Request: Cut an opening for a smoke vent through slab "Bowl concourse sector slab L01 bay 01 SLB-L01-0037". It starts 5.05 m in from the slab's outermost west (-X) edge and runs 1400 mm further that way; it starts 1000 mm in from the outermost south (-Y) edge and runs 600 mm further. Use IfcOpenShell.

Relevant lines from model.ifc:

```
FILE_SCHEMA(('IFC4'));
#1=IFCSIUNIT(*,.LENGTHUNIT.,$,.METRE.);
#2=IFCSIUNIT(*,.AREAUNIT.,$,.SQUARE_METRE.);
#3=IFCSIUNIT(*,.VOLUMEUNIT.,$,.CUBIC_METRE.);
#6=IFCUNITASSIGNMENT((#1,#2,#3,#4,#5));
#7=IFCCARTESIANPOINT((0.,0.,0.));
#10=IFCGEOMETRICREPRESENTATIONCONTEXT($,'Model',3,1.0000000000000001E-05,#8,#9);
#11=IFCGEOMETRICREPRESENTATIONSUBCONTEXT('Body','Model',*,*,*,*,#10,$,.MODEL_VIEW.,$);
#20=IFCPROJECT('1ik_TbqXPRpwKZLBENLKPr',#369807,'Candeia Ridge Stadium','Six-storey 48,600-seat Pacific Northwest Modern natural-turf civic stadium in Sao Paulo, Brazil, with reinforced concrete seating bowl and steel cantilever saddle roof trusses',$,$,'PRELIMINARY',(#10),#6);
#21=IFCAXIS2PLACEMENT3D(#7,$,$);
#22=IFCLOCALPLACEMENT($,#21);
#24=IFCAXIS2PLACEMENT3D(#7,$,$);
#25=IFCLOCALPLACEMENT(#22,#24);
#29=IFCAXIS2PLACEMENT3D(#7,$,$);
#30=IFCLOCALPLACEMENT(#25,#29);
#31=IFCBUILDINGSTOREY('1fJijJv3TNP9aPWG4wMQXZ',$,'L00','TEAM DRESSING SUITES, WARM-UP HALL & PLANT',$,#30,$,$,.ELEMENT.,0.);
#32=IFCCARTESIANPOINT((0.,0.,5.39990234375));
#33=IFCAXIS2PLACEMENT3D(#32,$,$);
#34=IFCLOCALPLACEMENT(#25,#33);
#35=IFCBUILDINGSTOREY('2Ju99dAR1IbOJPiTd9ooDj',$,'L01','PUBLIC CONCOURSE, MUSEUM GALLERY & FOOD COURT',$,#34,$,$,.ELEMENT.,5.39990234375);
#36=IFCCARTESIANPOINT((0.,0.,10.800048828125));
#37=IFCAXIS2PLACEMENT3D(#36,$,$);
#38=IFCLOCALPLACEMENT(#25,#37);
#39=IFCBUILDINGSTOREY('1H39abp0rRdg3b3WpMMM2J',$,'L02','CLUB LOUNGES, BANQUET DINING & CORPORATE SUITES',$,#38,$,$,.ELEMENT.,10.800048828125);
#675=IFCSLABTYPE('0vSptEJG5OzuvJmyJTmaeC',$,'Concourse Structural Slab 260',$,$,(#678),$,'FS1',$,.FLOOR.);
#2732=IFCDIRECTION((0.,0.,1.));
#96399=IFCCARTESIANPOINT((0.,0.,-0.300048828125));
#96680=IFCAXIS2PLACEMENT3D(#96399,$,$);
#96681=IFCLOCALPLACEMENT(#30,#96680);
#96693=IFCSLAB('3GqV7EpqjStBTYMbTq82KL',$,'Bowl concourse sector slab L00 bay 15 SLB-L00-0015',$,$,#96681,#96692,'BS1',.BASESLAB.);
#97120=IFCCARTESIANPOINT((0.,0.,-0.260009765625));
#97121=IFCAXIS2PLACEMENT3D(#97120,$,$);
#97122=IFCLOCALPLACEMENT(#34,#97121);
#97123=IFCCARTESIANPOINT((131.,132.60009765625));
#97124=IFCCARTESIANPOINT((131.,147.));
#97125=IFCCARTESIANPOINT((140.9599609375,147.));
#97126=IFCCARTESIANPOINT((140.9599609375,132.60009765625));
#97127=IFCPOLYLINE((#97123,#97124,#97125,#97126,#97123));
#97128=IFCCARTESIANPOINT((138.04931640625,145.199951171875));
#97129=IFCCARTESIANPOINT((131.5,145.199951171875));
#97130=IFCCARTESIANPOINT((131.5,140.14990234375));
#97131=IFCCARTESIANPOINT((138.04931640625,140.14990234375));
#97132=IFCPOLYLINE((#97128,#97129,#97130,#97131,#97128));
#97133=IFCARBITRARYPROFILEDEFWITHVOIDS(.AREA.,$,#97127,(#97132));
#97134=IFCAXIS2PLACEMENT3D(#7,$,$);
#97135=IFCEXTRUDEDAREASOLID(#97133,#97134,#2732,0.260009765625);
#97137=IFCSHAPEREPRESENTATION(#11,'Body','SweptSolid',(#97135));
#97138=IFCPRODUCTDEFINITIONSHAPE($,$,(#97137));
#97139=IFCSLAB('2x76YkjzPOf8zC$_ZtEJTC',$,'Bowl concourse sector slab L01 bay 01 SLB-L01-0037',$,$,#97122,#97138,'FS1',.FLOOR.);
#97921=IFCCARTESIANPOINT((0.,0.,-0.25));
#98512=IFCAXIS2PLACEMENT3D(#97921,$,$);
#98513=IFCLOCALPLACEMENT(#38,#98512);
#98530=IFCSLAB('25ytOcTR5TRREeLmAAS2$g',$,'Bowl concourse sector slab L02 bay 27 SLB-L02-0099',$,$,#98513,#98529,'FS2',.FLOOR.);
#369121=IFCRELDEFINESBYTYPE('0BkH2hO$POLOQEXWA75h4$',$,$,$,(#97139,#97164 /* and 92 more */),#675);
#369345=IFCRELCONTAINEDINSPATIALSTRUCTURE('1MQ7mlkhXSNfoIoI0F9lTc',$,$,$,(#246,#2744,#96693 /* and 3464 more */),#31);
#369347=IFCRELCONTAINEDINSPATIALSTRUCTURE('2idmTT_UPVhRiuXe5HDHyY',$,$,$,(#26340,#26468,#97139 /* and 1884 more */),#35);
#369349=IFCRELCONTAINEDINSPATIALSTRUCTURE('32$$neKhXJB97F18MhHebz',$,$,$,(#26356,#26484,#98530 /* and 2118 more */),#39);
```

```python
import numpy as np
import ifcopenshell
import ifcopenshell.api.feature
import ifcopenshell.api.geometry
import ifcopenshell.api.root
import ifcopenshell.geom
import ifcopenshell.util.placement
import ifcopenshell.util.representation
import ifcopenshell.util.shape
import ifcopenshell.util.unit

model = ifcopenshell.open("model.ifc")
unit_scale = ifcopenshell.util.unit.calculate_unit_scale(model)
settings = ifcopenshell.geom.settings()


def volume(element):
    """Net volume in cubic metres, openings subtracted."""
    shape = ifcopenshell.geom.create_shape(settings, element)
    return ifcopenshell.util.shape.get_volume(shape.geometry)


slab = model.by_guid("2x76YkjzPOf8zC$_ZtEJTC")
before = volume(slab)

# Extent in the slab's own axes, in metres. The edges named are its -X and -Y sides.
slab_shape = ifcopenshell.geom.create_shape(settings, slab)
vertices = ifcopenshell.util.shape.get_vertices(slab_shape.geometry)
x_min, y_min, bottom = vertices.min(axis=0)
top = vertices[:, 2].max()

opening = ifcopenshell.api.root.create_entity(model, ifc_class="IfcOpeningElement", name="Smoke vent opening", predefined_type="OPENING")
context = ifcopenshell.util.representation.get_context(model, "Model", "Body", "MODEL_VIEW")
width, depth = 1.4, 0.6
outline = [(0.0, 0.0), (width, 0.0), (width, depth), (0.0, depth), (0.0, 0.0)]
# Overshoot both faces by 50 mm so the cut is clean.
shape = ifcopenshell.api.geometry.add_slab_representation(
    model, context=context, depth=top - bottom + 0.1, polyline=outline
)
ifcopenshell.api.geometry.assign_representation(model, product=opening, representation=shape)

matrix = ifcopenshell.util.placement.get_local_placement(slab.ObjectPlacement)
matrix[:, 3] = matrix @ np.append(np.array([x_min + 5.05, y_min + 1, bottom - 0.05]) / unit_scale, 1.0)
ifcopenshell.api.geometry.edit_object_placement(model, product=opening, matrix=matrix, is_si=False)
ifcopenshell.api.feature.add_feature(model, feature=opening, element=slab)

after = volume(slab)

print(f"slab volume {before:.3f} -> {after:.3f} m3")

model.write("model_edited.ifc")
```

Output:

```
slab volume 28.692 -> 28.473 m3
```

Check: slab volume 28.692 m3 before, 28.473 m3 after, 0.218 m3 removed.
